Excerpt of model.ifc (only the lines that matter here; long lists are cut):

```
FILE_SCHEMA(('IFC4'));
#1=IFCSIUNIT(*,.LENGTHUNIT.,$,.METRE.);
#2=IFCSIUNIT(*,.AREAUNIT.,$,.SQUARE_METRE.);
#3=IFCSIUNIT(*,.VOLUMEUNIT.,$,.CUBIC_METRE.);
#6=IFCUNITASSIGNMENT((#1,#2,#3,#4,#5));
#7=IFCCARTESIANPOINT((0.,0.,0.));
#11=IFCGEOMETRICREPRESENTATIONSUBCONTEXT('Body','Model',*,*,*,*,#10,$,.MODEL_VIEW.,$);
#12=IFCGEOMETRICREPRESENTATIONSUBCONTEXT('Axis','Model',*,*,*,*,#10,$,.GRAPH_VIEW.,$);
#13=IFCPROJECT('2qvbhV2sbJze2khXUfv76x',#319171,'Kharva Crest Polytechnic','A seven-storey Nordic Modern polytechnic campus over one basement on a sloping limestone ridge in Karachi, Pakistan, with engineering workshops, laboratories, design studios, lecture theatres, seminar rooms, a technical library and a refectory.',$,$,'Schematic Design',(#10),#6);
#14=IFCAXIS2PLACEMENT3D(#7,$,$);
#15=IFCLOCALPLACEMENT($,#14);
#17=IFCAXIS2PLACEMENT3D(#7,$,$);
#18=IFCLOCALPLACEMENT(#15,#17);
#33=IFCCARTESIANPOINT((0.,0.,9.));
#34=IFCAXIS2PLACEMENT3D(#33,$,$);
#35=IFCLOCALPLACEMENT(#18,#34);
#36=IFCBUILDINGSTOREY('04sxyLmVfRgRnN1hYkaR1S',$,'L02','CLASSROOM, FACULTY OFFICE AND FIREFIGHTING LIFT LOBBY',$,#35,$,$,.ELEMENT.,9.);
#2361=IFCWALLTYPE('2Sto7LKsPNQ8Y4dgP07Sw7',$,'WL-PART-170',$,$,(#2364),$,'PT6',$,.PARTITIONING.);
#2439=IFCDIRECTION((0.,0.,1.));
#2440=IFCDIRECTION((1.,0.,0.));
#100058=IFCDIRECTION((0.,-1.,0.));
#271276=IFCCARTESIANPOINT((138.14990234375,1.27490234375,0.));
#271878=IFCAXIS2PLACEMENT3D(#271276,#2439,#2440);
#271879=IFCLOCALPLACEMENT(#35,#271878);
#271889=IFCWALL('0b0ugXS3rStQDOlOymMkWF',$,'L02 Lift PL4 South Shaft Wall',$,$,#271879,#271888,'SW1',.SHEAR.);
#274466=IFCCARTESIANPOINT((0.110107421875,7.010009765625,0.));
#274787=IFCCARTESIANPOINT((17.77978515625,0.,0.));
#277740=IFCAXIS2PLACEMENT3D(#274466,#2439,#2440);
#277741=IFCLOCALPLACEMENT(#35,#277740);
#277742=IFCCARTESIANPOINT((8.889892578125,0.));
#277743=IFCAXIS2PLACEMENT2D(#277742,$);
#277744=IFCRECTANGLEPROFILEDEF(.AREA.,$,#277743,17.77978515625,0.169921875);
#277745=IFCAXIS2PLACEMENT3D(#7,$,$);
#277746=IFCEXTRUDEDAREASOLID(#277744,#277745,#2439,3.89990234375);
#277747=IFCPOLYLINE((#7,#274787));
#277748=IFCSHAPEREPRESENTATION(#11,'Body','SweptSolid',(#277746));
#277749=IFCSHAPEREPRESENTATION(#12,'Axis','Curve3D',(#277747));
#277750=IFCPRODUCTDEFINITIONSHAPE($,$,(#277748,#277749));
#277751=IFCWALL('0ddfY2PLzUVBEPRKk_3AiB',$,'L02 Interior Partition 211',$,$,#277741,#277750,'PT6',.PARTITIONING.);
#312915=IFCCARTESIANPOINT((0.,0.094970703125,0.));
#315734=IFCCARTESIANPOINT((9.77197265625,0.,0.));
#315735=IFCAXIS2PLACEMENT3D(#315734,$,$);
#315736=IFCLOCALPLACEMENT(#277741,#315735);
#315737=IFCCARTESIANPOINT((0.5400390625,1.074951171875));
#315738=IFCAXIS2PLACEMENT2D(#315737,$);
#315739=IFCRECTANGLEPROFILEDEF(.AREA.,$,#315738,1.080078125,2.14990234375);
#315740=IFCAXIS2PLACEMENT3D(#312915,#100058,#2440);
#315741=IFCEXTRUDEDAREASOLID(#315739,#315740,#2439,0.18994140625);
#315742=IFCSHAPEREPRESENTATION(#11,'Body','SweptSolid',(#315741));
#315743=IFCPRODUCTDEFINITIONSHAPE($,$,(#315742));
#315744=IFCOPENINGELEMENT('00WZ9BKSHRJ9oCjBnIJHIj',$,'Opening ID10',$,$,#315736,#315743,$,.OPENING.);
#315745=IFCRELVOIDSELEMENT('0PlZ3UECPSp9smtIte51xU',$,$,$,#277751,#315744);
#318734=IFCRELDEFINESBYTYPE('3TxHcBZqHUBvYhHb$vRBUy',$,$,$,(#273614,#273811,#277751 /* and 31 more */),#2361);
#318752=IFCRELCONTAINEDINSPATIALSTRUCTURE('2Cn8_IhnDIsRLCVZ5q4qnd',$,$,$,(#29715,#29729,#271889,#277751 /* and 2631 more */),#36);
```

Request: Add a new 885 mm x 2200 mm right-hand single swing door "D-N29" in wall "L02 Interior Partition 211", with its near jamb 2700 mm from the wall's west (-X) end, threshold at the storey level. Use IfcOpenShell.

```python
import numpy as np
import ifcopenshell
import ifcopenshell.api.feature
import ifcopenshell.api.geometry
import ifcopenshell.api.root
import ifcopenshell.api.spatial
import ifcopenshell.geom
import ifcopenshell.util.element
import ifcopenshell.util.placement
import ifcopenshell.util.representation
import ifcopenshell.util.shape
import ifcopenshell.util.unit

model = ifcopenshell.open("model.ifc")
unit_scale = ifcopenshell.util.unit.calculate_unit_scale(model)
settings = ifcopenshell.geom.settings()


def volume(element):
    """Net volume in cubic metres, openings subtracted."""
    shape = ifcopenshell.geom.create_shape(settings, element)
    return ifcopenshell.util.shape.get_volume(shape.geometry)


wall = model.by_id(277751)
storey = ifcopenshell.util.element.get_container(wall, ifc_class="IfcBuildingStorey")
context = ifcopenshell.util.representation.get_context(model, "Model", "Body", "MODEL_VIEW")
before = volume(wall)

width, height, from_end, sill = 0.885, 2.2, 2.7, 0.0  # metres

# The wall runs along its own X axis, and the end named is its -X end.
wall_shape = ifcopenshell.geom.create_shape(settings, wall)
x, y, z = ifcopenshell.util.shape.get_vertices(wall_shape.geometry).T
start = x.min() + from_end
face, thickness = float(y.min()), float(y.max() - y.min())
wall_matrix = ifcopenshell.util.placement.get_local_placement(wall.ObjectPlacement)
level = ifcopenshell.util.placement.get_local_placement(storey.ObjectPlacement)[2, 3]


def in_wall(x, y):
    """Placement at x, y metres in the wall's axes, at sill height."""
    matrix = wall_matrix.copy()
    matrix[:, 3] = wall_matrix @ np.array([x / unit_scale, y / unit_scale, 0.0, 1.0])
    matrix[2, 3] = level + sill / unit_scale
    return matrix


# Opening: a box that overshoots both wall faces by 50 mm.
opening = ifcopenshell.api.root.create_entity(model, ifc_class="IfcOpeningElement", predefined_type="OPENING")
box = ifcopenshell.api.geometry.add_wall_representation(
    model, context=context, length=width, height=height, thickness=thickness + 0.1
)
ifcopenshell.api.geometry.assign_representation(model, product=opening, representation=box)
ifcopenshell.api.geometry.edit_object_placement(model, product=opening, matrix=in_wall(start, face - 0.05), is_si=False)
ifcopenshell.api.feature.add_feature(model, feature=opening, element=wall)

door = ifcopenshell.api.root.create_entity(model, ifc_class="IfcDoor", name="D-N29", predefined_type="DOOR")
door.OverallWidth, door.OverallHeight = width / unit_scale, height / unit_scale
door.OperationType = "SINGLE_SWING_RIGHT"
body = ifcopenshell.api.geometry.add_door_representation(
    model,
    context=context,
    overall_width=door.OverallWidth,
    overall_height=door.OverallHeight,
    operation_type="SINGLE_SWING_RIGHT",
    lining_properties={"LiningDepth": thickness / unit_scale, "ThresholdDepth": thickness / unit_scale},
)
ifcopenshell.api.geometry.assign_representation(model, product=door, representation=body)
ifcopenshell.api.spatial.assign_container(model, products=[door], relating_structure=storey)
ifcopenshell.api.feature.add_filling(model, opening=opening, element=door)

# The lining spans the wall, so the door starts at the wall face.
ifcopenshell.api.geometry.edit_object_placement(model, product=door, matrix=in_wall(start, face), is_si=False)

after = volume(wall)

print(f"wall volume {before:.3f} -> {after:.3f} m3")

model.write("model_rev.ifc")
```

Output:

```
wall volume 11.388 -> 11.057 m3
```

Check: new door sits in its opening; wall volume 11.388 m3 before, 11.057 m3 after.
